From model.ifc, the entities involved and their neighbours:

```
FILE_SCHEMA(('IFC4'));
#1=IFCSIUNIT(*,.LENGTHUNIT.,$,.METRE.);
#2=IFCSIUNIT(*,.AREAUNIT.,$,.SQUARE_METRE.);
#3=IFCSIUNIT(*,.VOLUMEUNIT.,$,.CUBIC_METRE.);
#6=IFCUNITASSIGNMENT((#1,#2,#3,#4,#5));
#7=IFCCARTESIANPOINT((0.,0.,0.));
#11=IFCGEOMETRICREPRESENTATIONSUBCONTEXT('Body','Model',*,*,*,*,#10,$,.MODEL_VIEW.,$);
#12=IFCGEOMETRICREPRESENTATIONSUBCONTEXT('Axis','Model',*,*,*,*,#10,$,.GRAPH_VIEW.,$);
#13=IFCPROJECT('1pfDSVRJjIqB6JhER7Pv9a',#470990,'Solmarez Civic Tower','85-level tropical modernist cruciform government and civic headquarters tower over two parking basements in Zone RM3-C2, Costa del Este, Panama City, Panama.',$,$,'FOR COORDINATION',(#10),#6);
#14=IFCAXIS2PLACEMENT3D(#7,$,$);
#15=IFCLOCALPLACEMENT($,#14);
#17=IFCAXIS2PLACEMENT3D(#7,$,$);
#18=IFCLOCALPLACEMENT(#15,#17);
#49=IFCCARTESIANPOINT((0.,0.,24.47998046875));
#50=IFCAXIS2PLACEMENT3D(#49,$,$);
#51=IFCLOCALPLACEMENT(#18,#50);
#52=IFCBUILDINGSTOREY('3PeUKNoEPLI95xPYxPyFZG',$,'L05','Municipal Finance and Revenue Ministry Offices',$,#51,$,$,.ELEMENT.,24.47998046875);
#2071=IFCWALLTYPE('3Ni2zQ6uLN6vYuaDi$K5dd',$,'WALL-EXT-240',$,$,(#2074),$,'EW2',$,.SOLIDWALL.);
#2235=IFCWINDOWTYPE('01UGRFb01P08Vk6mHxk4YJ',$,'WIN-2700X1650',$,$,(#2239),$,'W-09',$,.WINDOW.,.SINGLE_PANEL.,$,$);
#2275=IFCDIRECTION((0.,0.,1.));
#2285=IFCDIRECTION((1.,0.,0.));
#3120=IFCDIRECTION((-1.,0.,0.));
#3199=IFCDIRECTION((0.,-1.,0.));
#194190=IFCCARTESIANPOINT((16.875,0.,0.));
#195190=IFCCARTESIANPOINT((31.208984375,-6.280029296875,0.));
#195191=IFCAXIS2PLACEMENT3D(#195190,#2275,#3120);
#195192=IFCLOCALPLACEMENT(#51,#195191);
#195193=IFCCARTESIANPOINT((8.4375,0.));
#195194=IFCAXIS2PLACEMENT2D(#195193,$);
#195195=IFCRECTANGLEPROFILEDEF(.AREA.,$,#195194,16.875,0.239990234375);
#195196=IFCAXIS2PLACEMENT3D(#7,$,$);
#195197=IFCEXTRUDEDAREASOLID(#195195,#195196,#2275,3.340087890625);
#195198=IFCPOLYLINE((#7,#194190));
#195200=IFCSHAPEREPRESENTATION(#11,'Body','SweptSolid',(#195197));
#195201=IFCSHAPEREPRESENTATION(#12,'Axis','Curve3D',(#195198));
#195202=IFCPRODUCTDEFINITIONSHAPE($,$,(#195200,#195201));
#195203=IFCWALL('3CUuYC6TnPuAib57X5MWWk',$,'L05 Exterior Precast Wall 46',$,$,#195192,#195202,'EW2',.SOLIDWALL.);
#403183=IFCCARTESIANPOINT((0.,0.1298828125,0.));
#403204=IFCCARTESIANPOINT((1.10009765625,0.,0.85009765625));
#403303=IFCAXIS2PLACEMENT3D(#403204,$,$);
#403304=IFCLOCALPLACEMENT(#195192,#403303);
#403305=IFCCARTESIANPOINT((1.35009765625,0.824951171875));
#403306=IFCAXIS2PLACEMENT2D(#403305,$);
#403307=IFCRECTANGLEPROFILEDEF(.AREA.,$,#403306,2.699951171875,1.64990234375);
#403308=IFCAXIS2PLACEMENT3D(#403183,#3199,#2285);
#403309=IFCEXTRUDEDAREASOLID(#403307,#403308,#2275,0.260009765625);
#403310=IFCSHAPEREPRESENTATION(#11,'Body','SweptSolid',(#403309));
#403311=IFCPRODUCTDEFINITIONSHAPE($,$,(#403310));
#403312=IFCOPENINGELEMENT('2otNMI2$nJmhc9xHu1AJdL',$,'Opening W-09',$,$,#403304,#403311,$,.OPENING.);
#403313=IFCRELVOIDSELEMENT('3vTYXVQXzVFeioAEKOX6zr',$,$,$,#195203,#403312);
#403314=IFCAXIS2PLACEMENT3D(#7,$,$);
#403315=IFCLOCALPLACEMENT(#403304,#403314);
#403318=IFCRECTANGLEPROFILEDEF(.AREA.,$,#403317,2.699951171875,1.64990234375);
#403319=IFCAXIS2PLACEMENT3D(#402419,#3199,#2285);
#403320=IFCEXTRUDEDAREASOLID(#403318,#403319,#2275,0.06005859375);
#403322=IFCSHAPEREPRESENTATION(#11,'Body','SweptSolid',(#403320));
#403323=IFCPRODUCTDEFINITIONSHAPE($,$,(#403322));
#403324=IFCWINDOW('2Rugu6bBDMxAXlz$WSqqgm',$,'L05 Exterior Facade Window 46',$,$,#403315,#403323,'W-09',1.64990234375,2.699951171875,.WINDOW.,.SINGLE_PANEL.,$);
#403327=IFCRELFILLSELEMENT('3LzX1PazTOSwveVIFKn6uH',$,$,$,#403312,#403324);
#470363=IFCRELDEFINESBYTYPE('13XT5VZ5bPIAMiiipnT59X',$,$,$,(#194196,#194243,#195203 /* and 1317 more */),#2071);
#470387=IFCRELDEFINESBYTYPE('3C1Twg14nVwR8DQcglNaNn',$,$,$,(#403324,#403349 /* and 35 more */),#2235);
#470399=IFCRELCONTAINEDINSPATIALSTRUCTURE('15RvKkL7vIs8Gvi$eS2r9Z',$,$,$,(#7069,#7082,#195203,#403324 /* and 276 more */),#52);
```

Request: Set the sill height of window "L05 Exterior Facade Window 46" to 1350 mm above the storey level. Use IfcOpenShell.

```python
import numpy as np
import ifcopenshell
import ifcopenshell.api.geometry
import ifcopenshell.geom
import ifcopenshell.util.element
import ifcopenshell.util.placement
import ifcopenshell.util.shape
import ifcopenshell.util.unit

model = ifcopenshell.open("model.ifc")
unit_scale = ifcopenshell.util.unit.calculate_unit_scale(model)

window = model.by_id(403324)
opening = window.FillsVoids[0].RelatingOpeningElement
storey = ifcopenshell.util.element.get_container(window, ifc_class="IfcBuildingStorey")
level = ifcopenshell.util.placement.get_local_placement(storey.ObjectPlacement)[2, 3]

# The opening's origin need not be at the sill, so measure its lowest point.
shape = ifcopenshell.geom.create_shape(ifcopenshell.geom.settings(), opening)
bottom = ifcopenshell.util.shape.get_shape_bottom_elevation(shape, shape.geometry) / unit_scale
dz = level + 1.35 / unit_scale - bottom

shift = np.array([0.0, 0.0, dz])
# The window is placed relative to its opening, so it follows when the opening moves.
matrix = ifcopenshell.util.placement.get_local_placement(opening.ObjectPlacement)
matrix[:3, 3] += shift
ifcopenshell.api.geometry.edit_object_placement(
    model, product=opening, matrix=matrix, is_si=False, should_transform_children=True
)

print(f"moved by {dz * unit_scale:+.3f} m")

model.write("model-out.ifc")
```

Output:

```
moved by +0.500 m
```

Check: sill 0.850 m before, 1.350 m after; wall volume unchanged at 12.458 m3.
